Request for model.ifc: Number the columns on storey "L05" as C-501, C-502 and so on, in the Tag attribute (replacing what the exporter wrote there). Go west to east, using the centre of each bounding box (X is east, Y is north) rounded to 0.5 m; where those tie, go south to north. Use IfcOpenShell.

First a look at what the model holds.

```python
import ifcopenshell
import ifcopenshell.util.element
import ifcopenshell.util.placement

model = ifcopenshell.open("model.ifc")
print(model.schema)
storey = next(s for s in model.by_type("IfcBuildingStorey") if s.Name == "L05")
columns = [e for e in ifcopenshell.util.element.get_decomposition(storey) if e.is_a("IfcColumn")]
for e in sorted(columns, key=lambda e: e.id()):
    origin = ifcopenshell.util.placement.get_local_placement(e.ObjectPlacement)[:3, 3]
    print(e.id(), e.Tag, e.Name, origin.round(2) + 0.0, sep=" | ")
```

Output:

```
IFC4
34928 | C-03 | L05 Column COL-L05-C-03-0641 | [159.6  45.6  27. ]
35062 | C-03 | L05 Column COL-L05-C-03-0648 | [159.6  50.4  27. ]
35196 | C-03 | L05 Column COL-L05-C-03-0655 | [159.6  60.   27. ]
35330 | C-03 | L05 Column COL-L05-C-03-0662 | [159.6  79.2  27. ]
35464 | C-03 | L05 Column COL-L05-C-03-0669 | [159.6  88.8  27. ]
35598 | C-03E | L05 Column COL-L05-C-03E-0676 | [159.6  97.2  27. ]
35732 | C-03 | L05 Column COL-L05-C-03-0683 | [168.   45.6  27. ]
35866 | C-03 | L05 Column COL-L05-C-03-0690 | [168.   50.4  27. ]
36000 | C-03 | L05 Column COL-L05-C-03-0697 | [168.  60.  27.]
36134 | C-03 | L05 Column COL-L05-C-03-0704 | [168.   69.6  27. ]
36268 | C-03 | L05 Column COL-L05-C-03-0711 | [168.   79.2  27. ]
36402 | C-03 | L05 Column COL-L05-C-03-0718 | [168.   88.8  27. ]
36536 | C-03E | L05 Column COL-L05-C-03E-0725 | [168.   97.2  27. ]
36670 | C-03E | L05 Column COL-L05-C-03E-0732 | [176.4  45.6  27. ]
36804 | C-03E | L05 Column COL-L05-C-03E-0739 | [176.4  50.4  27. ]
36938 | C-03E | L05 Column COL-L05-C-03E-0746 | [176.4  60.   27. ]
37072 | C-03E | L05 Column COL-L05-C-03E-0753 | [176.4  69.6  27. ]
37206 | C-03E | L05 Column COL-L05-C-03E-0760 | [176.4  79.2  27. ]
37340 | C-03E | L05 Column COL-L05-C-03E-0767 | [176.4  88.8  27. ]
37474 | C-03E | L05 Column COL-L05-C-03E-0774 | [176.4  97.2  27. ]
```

```python
import ifcopenshell
import ifcopenshell.geom
import ifcopenshell.util.element
import ifcopenshell.util.shape

model = ifcopenshell.open("model.ifc")
settings = ifcopenshell.geom.settings()
settings.set("use-world-coords", True)


def centre(element):
    shape = ifcopenshell.geom.create_shape(settings, element)
    return ifcopenshell.util.shape.get_bbox_centroid(shape.geometry)


storey = next(s for s in model.by_type("IfcBuildingStorey") if s.Name == "L05")
columns = [e for e in ifcopenshell.util.element.get_decomposition(storey) if e.is_a("IfcColumn")]

# Insertion points can sit at a corner or the storey origin, so sort by the geometry (in metres).
centres = {e: centre(e) for e in columns}
columns.sort(key=lambda e: (round(centres[e][0] / 0.5), centres[e][1]))

for i, e in enumerate(columns, start=1):
    number = f"C-5{i:02d}"
    e.Tag = number
    print(e.id(), number)

model.write("model_edited.ifc")
```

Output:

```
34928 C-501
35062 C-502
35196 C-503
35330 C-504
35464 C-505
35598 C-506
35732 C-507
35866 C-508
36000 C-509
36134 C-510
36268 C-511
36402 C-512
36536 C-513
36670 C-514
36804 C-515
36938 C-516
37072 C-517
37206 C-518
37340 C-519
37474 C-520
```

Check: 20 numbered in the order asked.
